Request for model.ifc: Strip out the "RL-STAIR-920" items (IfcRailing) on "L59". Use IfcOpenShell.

First a look at what the model holds.

```python
import ifcopenshell
import ifcopenshell.util.element

model = ifcopenshell.open("model.ifc")
print(model.schema)
storey = next(s for s in model.by_type("IfcBuildingStorey") if s.Name == "L59")
railings = [e for e in ifcopenshell.util.element.get_decomposition(storey) if e.is_a("IfcRailing")]
seen = {}
for e in railings:
    element_type = ifcopenshell.util.element.get_type(e)
    name = element_type.Name if element_type not in (None, e) else None
    seen[name] = seen.get(name, 0) + 1
for name, count in sorted(seen.items(), key=str):
    print(count, "x", name)
```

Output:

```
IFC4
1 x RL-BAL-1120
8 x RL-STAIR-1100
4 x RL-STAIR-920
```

```python
import ifcopenshell
import ifcopenshell.api.root
import ifcopenshell.util.element

model = ifcopenshell.open("model.ifc")

storey = next(s for s in model.by_type("IfcBuildingStorey") if s.Name == "L59")
railings = [e for e in ifcopenshell.util.element.get_decomposition(storey) if e.is_a("IfcRailing")]
targets = [e for e in railings if (t := ifcopenshell.util.element.get_type(e)) not in (None, e) and t.Name == "RL-STAIR-920"]

for e in targets:
    ifcopenshell.api.root.remove_product(model, product=e)
print(len(targets), "removed")

model.write("model_edited.ifc")
```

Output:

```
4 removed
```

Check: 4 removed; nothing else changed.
